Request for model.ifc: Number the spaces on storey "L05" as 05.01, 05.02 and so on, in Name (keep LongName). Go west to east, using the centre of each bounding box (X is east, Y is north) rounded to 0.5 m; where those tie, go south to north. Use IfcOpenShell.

First a look at what the model holds.

```python
import ifcopenshell
import ifcopenshell.util.element
import ifcopenshell.util.placement

model = ifcopenshell.open("model.ifc")
print(model.schema)
storey = next(s for s in model.by_type("IfcBuildingStorey") if s.Name == "L05")
spaces = [e for e in ifcopenshell.util.element.get_decomposition(storey) if e.is_a("IfcSpace")]
for e in sorted(spaces, key=lambda e: e.id()):
    origin = ifcopenshell.util.placement.get_local_placement(e.ObjectPlacement)[:3, 3]
    print(e.id(), e.Name, e.LongName, origin.round(2) + 0.0, sep=" | ")
```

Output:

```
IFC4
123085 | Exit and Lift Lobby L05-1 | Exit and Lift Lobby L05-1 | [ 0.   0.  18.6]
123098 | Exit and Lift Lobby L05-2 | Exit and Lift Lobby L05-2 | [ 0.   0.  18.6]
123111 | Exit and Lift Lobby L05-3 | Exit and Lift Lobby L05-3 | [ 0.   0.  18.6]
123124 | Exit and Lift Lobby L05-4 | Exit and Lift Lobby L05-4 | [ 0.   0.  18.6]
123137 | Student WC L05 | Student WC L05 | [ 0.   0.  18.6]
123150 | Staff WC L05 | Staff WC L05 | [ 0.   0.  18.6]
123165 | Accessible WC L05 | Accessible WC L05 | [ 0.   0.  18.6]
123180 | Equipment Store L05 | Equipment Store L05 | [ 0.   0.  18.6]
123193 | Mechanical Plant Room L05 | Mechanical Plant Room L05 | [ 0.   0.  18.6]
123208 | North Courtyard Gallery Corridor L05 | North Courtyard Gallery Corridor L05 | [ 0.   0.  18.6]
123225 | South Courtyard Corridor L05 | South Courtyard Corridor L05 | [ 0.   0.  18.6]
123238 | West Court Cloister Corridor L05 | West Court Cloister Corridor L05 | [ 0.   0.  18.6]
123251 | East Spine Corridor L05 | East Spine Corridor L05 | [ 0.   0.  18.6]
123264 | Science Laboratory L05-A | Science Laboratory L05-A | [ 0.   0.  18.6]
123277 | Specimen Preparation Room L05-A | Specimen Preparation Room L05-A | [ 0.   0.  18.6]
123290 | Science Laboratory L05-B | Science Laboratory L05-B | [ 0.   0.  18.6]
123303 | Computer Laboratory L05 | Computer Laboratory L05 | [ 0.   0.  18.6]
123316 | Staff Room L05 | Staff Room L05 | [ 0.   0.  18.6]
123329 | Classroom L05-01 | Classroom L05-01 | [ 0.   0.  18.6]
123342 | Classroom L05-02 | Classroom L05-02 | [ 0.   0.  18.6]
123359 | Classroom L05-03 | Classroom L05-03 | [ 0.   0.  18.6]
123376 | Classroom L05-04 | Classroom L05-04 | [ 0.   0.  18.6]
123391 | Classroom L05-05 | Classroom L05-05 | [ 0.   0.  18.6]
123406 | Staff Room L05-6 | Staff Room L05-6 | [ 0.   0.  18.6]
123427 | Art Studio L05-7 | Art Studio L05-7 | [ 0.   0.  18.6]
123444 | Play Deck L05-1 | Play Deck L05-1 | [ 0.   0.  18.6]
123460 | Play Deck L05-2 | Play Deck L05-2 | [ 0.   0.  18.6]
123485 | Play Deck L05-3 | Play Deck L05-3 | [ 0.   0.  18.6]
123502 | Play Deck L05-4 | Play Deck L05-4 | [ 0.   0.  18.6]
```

```python
import ifcopenshell
import ifcopenshell.geom
import ifcopenshell.util.element
import ifcopenshell.util.shape

model = ifcopenshell.open("model.ifc")
settings = ifcopenshell.geom.settings()
settings.set("use-world-coords", True)


def centre(element):
    shape = ifcopenshell.geom.create_shape(settings, element)
    return ifcopenshell.util.shape.get_bbox_centroid(shape.geometry)


storey = next(s for s in model.by_type("IfcBuildingStorey") if s.Name == "L05")
spaces = [e for e in ifcopenshell.util.element.get_decomposition(storey) if e.is_a("IfcSpace")]

# Insertion points can sit at a corner or the storey origin, so sort by the geometry (in metres).
centres = {e: centre(e) for e in spaces}
spaces.sort(key=lambda e: (round(centres[e][0] / 0.5), centres[e][1]))

for i, e in enumerate(spaces, start=1):
    number = f"05.{i:02d}"
    e.Name = number
    print(e.id(), number)

model.write("model_edited.ifc")
```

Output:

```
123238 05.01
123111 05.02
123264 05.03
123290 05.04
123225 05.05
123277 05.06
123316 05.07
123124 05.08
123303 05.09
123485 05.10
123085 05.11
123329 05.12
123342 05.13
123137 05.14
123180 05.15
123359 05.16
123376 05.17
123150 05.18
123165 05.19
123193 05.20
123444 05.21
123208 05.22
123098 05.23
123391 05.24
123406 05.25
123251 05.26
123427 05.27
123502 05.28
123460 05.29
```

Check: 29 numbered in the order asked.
